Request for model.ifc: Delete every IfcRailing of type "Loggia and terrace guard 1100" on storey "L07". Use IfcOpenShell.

First a look at what the model holds.

```python
import ifcopenshell
import ifcopenshell.util.element

model = ifcopenshell.open("model.ifc")
print(model.schema)
storey = next(s for s in model.by_type("IfcBuildingStorey") if s.Name == "L07")
railings = [e for e in ifcopenshell.util.element.get_decomposition(storey) if e.is_a("IfcRailing")]
seen = {}
for e in railings:
    element_type = ifcopenshell.util.element.get_type(e)
    name = element_type.Name if element_type not in (None, e) else None
    seen[name] = seen.get(name, 0) + 1
for name, count in sorted(seen.items(), key=str):
    print(count, "x", name)
```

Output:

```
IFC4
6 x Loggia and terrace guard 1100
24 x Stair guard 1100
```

```python
import ifcopenshell
import ifcopenshell.api.root
import ifcopenshell.util.element

model = ifcopenshell.open("model.ifc")

storey = next(s for s in model.by_type("IfcBuildingStorey") if s.Name == "L07")
railings = [e for e in ifcopenshell.util.element.get_decomposition(storey) if e.is_a("IfcRailing")]
targets = [e for e in railings if (t := ifcopenshell.util.element.get_type(e)) not in (None, e) and t.Name == "Loggia and terrace guard 1100"]

for e in targets:
    ifcopenshell.api.root.remove_product(model, product=e)
print(len(targets), "removed")

model.write("model-out.ifc")
```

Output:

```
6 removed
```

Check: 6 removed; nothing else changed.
